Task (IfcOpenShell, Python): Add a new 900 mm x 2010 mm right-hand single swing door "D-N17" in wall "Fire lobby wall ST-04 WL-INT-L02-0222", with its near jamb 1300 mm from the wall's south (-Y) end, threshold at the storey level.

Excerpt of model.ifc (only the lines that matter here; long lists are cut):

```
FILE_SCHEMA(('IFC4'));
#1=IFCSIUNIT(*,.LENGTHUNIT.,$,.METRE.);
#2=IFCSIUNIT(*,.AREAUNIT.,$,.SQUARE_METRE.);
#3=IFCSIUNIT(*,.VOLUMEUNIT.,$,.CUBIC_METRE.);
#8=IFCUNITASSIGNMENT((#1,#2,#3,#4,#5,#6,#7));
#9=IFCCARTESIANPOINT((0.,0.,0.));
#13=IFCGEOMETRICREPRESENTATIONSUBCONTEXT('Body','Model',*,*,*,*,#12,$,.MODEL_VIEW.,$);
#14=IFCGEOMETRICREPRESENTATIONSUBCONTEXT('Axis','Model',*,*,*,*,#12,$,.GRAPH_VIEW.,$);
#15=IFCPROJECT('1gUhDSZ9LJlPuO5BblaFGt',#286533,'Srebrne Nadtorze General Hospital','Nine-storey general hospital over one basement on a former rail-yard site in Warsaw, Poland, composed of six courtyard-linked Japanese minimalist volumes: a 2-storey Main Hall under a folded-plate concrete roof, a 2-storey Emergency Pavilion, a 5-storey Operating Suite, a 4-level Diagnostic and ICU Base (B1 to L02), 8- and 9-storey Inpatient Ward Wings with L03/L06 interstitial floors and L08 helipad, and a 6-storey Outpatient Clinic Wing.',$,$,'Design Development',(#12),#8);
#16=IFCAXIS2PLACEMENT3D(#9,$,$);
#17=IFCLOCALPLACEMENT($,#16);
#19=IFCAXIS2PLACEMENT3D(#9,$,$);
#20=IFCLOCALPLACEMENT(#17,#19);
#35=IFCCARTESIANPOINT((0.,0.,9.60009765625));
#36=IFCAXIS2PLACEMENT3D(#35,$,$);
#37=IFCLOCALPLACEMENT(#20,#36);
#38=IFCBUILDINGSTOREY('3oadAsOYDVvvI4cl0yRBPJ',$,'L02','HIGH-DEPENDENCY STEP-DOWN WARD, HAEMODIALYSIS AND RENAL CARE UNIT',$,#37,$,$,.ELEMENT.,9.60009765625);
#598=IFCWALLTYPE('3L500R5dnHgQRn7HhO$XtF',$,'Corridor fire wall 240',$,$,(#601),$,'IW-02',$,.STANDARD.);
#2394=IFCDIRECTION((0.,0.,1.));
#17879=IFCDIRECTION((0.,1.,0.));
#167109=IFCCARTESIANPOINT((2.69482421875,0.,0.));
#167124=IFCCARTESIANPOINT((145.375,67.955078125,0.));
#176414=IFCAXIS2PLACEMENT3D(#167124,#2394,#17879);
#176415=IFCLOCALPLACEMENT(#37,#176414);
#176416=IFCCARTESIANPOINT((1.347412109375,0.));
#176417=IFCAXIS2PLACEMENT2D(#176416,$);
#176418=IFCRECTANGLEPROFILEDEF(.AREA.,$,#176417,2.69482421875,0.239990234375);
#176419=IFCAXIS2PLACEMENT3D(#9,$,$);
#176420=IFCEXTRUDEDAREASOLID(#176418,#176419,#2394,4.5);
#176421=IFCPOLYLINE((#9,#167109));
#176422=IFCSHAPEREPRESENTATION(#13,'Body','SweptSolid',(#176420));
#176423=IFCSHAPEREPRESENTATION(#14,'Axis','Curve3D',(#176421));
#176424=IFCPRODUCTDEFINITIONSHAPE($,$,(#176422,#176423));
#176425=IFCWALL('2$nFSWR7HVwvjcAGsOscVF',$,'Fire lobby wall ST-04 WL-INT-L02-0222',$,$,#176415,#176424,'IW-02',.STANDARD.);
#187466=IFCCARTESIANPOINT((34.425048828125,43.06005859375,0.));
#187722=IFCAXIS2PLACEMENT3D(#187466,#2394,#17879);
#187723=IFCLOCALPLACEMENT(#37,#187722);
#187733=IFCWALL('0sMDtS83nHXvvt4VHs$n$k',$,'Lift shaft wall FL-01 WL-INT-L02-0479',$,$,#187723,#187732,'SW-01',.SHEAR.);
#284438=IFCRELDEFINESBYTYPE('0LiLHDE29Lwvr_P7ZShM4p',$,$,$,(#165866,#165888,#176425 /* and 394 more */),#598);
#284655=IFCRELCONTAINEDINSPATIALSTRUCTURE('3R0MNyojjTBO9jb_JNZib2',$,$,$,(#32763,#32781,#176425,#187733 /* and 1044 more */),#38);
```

```python
import numpy as np
import ifcopenshell
import ifcopenshell.api.feature
import ifcopenshell.api.geometry
import ifcopenshell.api.root
import ifcopenshell.api.spatial
import ifcopenshell.geom
import ifcopenshell.util.element
import ifcopenshell.util.placement
import ifcopenshell.util.representation
import ifcopenshell.util.shape
import ifcopenshell.util.unit

model = ifcopenshell.open("model.ifc")
unit_scale = ifcopenshell.util.unit.calculate_unit_scale(model)
settings = ifcopenshell.geom.settings()


def volume(element):
    """Net volume in cubic metres, openings subtracted."""
    shape = ifcopenshell.geom.create_shape(settings, element)
    return ifcopenshell.util.shape.get_volume(shape.geometry)


wall = model.by_id(176425)
storey = ifcopenshell.util.element.get_container(wall, ifc_class="IfcBuildingStorey")
context = ifcopenshell.util.representation.get_context(model, "Model", "Body", "MODEL_VIEW")
before = volume(wall)

width, height, from_end, sill = 0.9, 2.01, 1.3, 0.0  # metres

# The wall runs along its own X axis, and the end named is its -X end.
wall_shape = ifcopenshell.geom.create_shape(settings, wall)
x, y, z = ifcopenshell.util.shape.get_vertices(wall_shape.geometry).T
start = x.min() + from_end
face, thickness = float(y.min()), float(y.max() - y.min())
wall_matrix = ifcopenshell.util.placement.get_local_placement(wall.ObjectPlacement)
level = ifcopenshell.util.placement.get_local_placement(storey.ObjectPlacement)[2, 3]


def in_wall(x, y):
    """Placement at x, y metres in the wall's axes, at sill height."""
    matrix = wall_matrix.copy()
    matrix[:, 3] = wall_matrix @ np.array([x / unit_scale, y / unit_scale, 0.0, 1.0])
    matrix[2, 3] = level + sill / unit_scale
    return matrix


# Opening: a box that overshoots both wall faces by 50 mm.
opening = ifcopenshell.api.root.create_entity(model, ifc_class="IfcOpeningElement", predefined_type="OPENING")
box = ifcopenshell.api.geometry.add_wall_representation(
    model, context=context, length=width, height=height, thickness=thickness + 0.1
)
ifcopenshell.api.geometry.assign_representation(model, product=opening, representation=box)
ifcopenshell.api.geometry.edit_object_placement(model, product=opening, matrix=in_wall(start, face - 0.05), is_si=False)
ifcopenshell.api.feature.add_feature(model, feature=opening, element=wall)

door = ifcopenshell.api.root.create_entity(model, ifc_class="IfcDoor", name="D-N17", predefined_type="DOOR")
door.OverallWidth, door.OverallHeight = width / unit_scale, height / unit_scale
door.OperationType = "SINGLE_SWING_RIGHT"
body = ifcopenshell.api.geometry.add_door_representation(
    model,
    context=context,
    overall_width=door.OverallWidth,
    overall_height=door.OverallHeight,
    operation_type="SINGLE_SWING_RIGHT",
    lining_properties={"LiningDepth": thickness / unit_scale, "ThresholdDepth": thickness / unit_scale},
)
ifcopenshell.api.geometry.assign_representation(model, product=door, representation=body)
ifcopenshell.api.spatial.assign_container(model, products=[door], relating_structure=storey)
ifcopenshell.api.feature.add_filling(model, opening=opening, element=door)

# The lining spans the wall, so the door starts at the wall face.
ifcopenshell.api.geometry.edit_object_placement(model, product=door, matrix=in_wall(start, face), is_si=False)

after = volume(wall)

print(f"wall volume {before:.3f} -> {after:.3f} m3")

model.write("model_v2.ifc")
```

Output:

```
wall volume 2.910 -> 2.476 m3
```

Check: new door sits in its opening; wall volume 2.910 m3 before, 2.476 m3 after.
